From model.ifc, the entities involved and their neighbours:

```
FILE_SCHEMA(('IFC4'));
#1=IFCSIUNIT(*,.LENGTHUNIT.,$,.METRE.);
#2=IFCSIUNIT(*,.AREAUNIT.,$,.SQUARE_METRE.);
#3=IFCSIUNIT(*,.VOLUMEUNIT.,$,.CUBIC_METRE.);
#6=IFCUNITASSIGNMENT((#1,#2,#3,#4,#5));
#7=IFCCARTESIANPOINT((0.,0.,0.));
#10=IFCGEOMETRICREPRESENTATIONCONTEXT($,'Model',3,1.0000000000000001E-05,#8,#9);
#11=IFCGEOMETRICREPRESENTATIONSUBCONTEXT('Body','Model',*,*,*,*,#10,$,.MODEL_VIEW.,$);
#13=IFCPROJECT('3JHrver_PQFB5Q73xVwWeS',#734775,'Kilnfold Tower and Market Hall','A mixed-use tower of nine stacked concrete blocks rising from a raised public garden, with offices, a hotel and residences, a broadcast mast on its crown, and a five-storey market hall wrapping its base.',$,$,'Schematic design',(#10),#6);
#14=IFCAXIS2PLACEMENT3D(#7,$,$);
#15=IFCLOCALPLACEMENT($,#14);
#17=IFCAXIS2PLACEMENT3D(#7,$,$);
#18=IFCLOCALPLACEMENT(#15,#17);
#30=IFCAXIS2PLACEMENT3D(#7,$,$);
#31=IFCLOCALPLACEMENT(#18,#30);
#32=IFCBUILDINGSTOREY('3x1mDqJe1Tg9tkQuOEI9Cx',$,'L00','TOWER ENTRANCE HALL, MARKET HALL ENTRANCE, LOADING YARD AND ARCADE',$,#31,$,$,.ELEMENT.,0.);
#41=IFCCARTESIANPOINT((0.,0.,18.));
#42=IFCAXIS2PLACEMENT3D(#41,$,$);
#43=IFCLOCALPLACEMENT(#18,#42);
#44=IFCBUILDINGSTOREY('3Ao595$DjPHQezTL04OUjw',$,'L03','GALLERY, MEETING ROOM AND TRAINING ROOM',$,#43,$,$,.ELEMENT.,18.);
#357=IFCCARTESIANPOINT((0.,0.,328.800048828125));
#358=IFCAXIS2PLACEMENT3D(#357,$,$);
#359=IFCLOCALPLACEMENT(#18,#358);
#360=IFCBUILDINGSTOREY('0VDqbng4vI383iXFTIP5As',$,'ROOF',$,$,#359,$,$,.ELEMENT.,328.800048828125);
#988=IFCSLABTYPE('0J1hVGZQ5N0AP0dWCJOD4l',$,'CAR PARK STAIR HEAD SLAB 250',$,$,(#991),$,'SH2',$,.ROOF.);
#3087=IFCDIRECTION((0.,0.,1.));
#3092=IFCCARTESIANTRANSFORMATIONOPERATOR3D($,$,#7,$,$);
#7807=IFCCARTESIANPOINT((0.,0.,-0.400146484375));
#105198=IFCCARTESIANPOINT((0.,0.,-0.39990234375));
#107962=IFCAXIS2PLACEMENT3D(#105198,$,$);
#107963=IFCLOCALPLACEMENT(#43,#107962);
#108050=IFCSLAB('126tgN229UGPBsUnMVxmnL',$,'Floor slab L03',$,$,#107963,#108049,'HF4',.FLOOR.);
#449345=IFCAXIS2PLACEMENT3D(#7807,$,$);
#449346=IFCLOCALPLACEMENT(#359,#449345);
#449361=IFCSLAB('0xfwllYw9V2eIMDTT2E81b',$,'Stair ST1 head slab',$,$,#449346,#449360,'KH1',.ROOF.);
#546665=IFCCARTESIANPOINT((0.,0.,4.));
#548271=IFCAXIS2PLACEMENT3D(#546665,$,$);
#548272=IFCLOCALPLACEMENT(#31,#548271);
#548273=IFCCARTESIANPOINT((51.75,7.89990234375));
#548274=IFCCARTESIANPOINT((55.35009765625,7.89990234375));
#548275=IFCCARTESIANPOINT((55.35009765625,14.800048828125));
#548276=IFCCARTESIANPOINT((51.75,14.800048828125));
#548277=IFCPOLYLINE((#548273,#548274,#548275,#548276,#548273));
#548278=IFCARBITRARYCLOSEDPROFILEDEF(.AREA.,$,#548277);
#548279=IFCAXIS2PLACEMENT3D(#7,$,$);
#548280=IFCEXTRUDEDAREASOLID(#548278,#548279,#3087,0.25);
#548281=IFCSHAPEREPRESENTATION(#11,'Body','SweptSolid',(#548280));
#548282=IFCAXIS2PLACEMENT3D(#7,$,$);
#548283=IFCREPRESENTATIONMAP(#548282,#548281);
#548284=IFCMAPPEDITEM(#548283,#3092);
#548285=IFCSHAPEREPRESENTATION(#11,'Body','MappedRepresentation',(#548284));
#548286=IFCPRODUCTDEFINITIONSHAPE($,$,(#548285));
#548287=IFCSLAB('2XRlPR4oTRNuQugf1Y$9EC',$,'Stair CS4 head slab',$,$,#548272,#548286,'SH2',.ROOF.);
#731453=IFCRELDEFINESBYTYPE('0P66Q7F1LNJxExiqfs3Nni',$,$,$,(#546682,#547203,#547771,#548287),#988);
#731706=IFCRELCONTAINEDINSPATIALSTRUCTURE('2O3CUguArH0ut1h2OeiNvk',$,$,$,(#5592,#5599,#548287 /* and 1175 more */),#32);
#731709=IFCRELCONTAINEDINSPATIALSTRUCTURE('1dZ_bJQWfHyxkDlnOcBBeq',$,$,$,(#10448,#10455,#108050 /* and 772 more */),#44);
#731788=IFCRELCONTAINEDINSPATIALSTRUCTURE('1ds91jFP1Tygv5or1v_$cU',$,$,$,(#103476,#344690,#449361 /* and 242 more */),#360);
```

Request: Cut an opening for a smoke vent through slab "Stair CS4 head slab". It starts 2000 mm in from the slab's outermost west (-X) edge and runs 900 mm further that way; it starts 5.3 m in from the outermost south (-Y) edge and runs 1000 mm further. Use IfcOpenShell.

```python
import numpy as np
import ifcopenshell
import ifcopenshell.api.feature
import ifcopenshell.api.geometry
import ifcopenshell.api.root
import ifcopenshell.geom
import ifcopenshell.util.placement
import ifcopenshell.util.representation
import ifcopenshell.util.shape
import ifcopenshell.util.unit

model = ifcopenshell.open("model.ifc")
unit_scale = ifcopenshell.util.unit.calculate_unit_scale(model)
settings = ifcopenshell.geom.settings()


def volume(element):
    """Net volume in cubic metres, openings subtracted."""
    shape = ifcopenshell.geom.create_shape(settings, element)
    return ifcopenshell.util.shape.get_volume(shape.geometry)


slab = model.by_id(548287)
before = volume(slab)

# Extent in the slab's own axes, in metres. The edges named are its -X and -Y sides.
slab_shape = ifcopenshell.geom.create_shape(settings, slab)
vertices = ifcopenshell.util.shape.get_vertices(slab_shape.geometry)
x_min, y_min, bottom = vertices.min(axis=0)
top = vertices[:, 2].max()

opening = ifcopenshell.api.root.create_entity(model, ifc_class="IfcOpeningElement", name="Smoke vent opening", predefined_type="OPENING")
context = ifcopenshell.util.representation.get_context(model, "Model", "Body", "MODEL_VIEW")
width, depth = 0.9, 1
outline = [(0.0, 0.0), (width, 0.0), (width, depth), (0.0, depth), (0.0, 0.0)]
# Overshoot both faces by 50 mm so the cut is clean.
shape = ifcopenshell.api.geometry.add_slab_representation(
    model, context=context, depth=top - bottom + 0.1, polyline=outline
)
ifcopenshell.api.geometry.assign_representation(model, product=opening, representation=shape)

matrix = ifcopenshell.util.placement.get_local_placement(slab.ObjectPlacement)
matrix[:, 3] = matrix @ np.append(np.array([x_min + 2, y_min + 5.3, bottom - 0.05]) / unit_scale, 1.0)
ifcopenshell.api.geometry.edit_object_placement(model, product=opening, matrix=matrix, is_si=False)
ifcopenshell.api.feature.add_feature(model, feature=opening, element=slab)

after = volume(slab)

print(f"slab volume {before:.3f} -> {after:.3f} m3")

model.write("model_rev.ifc")
```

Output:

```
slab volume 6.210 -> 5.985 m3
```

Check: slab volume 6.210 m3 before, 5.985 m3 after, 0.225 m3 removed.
